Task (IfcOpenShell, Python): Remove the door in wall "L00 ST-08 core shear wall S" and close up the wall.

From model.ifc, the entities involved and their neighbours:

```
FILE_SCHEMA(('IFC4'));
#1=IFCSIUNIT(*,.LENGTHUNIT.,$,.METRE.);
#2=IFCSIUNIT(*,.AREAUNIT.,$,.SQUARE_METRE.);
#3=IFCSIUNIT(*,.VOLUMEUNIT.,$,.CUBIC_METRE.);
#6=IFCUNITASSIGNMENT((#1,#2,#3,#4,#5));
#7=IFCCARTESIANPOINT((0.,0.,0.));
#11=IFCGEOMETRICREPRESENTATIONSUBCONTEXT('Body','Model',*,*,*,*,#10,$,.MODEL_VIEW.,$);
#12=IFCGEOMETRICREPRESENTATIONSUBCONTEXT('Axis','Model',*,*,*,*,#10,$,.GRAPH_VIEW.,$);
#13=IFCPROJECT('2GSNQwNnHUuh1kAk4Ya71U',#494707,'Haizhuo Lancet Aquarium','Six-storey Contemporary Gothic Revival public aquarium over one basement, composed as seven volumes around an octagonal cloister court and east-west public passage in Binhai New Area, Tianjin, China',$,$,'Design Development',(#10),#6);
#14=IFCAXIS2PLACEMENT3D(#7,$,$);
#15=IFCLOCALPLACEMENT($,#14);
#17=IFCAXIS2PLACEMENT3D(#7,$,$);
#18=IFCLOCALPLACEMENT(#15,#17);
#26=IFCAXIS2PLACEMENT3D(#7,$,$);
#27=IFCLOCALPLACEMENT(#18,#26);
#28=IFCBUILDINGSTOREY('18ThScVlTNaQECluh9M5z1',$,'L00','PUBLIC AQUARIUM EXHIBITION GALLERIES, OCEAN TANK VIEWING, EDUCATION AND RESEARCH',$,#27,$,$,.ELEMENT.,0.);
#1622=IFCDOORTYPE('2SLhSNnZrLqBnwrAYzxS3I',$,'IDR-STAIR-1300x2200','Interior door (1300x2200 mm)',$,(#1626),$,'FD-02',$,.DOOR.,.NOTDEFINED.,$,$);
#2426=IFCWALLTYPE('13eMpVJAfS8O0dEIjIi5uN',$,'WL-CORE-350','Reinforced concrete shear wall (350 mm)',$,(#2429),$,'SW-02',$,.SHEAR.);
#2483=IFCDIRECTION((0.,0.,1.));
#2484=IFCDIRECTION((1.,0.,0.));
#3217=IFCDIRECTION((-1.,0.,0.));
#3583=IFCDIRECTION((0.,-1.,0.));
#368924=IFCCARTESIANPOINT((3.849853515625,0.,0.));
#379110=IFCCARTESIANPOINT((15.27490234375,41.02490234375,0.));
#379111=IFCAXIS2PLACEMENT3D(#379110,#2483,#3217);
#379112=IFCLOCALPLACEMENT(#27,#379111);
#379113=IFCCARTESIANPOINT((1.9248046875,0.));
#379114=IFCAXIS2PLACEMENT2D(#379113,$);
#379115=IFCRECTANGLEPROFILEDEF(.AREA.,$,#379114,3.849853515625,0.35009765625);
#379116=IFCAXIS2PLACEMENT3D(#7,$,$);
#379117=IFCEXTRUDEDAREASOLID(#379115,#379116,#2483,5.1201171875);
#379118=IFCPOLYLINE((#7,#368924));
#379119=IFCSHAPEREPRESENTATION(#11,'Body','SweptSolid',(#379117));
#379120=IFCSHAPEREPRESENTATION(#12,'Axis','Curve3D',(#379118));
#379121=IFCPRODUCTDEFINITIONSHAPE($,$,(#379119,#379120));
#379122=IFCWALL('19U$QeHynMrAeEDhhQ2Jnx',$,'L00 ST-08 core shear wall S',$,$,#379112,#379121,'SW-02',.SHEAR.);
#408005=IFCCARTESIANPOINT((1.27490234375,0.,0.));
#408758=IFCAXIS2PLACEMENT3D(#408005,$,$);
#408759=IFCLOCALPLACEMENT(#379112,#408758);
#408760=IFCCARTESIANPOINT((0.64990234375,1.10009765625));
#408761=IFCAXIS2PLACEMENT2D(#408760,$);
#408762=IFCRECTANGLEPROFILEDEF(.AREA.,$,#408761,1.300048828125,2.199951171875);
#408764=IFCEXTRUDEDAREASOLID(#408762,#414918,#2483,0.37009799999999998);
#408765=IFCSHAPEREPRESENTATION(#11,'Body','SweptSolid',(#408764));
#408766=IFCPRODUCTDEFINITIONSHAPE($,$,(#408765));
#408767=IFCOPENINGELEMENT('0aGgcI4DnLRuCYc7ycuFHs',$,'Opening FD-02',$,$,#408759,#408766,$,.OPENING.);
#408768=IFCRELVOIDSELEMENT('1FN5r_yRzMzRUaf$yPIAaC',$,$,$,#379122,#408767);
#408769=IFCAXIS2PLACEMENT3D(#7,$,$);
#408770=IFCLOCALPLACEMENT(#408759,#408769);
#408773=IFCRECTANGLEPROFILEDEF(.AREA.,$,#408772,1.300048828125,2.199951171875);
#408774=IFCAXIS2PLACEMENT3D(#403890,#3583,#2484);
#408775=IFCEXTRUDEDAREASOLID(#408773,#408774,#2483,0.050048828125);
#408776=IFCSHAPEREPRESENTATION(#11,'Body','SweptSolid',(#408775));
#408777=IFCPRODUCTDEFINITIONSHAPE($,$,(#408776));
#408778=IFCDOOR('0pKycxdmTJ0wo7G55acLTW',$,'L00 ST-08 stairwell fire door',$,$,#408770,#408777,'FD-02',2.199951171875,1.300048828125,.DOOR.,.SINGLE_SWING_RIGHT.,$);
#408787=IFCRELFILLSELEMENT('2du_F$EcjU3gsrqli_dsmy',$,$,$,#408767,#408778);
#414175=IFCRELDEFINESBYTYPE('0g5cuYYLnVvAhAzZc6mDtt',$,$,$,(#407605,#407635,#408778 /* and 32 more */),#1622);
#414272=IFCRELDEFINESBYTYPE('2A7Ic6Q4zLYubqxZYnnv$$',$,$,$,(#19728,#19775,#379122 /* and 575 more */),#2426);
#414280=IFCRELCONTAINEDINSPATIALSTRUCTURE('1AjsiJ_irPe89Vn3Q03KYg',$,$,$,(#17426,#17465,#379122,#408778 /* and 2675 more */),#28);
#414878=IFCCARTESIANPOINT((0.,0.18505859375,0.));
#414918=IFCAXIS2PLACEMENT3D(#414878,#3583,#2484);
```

```python
import ifcopenshell
import ifcopenshell.api.feature
import ifcopenshell.api.root
import ifcopenshell.geom
import ifcopenshell.util.shape

model = ifcopenshell.open("model.ifc")
settings = ifcopenshell.geom.settings()


def volume(element):
    """Net volume in cubic metres, openings subtracted."""
    shape = ifcopenshell.geom.create_shape(settings, element)
    return ifcopenshell.util.shape.get_volume(shape.geometry)


door = model.by_id(408778)
opening = door.FillsVoids[0].RelatingOpeningElement
wall = opening.VoidsElements[0].RelatingBuildingElement
before = volume(wall)

ifcopenshell.api.root.remove_product(model, product=door)
ifcopenshell.api.feature.remove_feature(model, feature=opening)

after = volume(wall)

print(f"wall volume {before:.3f} -> {after:.3f} m3")

model.write("model_updated.ifc")
```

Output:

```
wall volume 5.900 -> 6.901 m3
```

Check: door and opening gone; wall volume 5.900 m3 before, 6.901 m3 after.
